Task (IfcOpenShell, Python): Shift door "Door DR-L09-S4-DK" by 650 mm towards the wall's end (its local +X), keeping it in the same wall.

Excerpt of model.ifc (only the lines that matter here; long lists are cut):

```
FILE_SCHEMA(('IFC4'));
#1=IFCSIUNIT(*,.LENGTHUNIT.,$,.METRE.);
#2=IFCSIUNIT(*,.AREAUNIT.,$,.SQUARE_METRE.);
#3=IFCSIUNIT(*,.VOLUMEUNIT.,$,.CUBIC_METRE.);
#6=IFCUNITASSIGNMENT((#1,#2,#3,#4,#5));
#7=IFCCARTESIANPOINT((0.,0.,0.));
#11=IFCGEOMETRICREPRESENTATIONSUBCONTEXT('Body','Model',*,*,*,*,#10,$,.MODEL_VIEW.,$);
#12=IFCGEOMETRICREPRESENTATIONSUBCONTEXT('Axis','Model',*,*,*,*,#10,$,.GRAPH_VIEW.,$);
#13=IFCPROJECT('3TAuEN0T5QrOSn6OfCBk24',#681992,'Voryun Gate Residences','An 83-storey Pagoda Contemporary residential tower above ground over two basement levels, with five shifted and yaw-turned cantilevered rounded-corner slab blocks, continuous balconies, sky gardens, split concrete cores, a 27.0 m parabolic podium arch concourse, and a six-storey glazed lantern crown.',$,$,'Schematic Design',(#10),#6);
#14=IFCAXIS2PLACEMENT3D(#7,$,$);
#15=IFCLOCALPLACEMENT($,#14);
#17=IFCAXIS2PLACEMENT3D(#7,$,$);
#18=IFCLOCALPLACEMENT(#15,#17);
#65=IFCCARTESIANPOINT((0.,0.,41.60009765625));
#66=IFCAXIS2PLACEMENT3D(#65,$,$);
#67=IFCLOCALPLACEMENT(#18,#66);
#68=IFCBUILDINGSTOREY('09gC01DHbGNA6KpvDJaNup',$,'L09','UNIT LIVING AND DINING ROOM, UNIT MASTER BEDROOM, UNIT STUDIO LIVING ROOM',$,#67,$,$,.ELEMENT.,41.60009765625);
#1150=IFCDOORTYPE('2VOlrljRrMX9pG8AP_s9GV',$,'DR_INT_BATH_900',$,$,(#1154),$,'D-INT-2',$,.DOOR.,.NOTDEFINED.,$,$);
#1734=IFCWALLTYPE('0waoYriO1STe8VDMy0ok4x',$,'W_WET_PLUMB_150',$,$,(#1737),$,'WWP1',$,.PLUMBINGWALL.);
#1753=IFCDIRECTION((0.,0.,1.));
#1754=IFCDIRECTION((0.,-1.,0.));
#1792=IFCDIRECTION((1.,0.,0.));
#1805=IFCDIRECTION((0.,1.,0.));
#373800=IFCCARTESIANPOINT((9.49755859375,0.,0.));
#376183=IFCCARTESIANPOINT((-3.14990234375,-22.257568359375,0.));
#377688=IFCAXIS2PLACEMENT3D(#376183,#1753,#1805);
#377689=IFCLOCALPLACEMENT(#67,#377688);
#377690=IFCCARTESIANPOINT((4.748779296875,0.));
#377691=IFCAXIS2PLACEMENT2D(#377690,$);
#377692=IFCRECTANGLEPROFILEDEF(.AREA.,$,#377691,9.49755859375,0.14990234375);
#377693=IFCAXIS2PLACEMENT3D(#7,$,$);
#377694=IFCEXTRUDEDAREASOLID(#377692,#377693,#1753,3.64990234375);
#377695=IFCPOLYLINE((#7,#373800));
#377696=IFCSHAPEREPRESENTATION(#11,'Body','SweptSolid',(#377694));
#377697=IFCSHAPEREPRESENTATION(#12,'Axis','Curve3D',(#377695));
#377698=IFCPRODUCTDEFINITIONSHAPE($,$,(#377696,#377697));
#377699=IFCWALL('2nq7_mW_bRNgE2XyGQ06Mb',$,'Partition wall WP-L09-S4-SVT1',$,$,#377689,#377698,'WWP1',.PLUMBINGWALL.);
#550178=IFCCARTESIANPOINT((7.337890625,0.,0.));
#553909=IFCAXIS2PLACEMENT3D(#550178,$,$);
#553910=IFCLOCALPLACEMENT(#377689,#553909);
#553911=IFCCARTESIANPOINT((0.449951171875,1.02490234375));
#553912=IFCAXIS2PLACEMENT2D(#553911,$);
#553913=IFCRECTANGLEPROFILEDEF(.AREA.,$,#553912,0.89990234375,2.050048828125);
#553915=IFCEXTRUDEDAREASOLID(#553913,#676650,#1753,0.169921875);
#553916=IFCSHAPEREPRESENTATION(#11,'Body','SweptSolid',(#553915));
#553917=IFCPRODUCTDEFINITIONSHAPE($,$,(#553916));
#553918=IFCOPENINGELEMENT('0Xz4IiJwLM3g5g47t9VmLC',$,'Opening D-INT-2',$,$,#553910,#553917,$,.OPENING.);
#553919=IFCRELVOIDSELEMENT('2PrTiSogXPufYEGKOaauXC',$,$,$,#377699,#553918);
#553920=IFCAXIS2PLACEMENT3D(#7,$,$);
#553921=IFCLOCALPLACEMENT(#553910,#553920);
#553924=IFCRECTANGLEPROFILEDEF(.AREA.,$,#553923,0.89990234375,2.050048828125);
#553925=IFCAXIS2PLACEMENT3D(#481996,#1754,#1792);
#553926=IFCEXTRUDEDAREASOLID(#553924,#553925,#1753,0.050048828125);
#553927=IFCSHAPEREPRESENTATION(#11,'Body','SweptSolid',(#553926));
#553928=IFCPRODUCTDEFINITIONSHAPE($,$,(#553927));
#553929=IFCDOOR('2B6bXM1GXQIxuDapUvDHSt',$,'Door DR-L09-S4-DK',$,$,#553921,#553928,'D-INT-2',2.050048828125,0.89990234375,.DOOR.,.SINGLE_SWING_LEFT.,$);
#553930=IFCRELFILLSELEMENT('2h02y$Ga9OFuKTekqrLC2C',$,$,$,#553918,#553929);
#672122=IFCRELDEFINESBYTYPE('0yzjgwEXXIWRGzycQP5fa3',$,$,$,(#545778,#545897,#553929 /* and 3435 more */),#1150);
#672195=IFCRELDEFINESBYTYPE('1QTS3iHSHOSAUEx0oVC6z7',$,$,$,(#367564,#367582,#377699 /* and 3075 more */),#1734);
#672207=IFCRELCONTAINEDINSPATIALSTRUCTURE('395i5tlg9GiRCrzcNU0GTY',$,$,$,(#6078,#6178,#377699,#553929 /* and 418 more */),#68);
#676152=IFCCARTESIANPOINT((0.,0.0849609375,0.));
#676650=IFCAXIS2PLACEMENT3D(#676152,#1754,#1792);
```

```python
import ifcopenshell
import ifcopenshell.api.geometry
import ifcopenshell.util.placement
import ifcopenshell.util.unit

model = ifcopenshell.open("model.ifc")
unit_scale = ifcopenshell.util.unit.calculate_unit_scale(model)

door = model.by_guid("2B6bXM1GXQIxuDapUvDHSt")
opening = door.FillsVoids[0].RelatingOpeningElement
wall = opening.VoidsElements[0].RelatingBuildingElement

wall_matrix = ifcopenshell.util.placement.get_local_placement(wall.ObjectPlacement)
shift = wall_matrix[:3, 0] * 0.65 / unit_scale
before = ifcopenshell.util.placement.get_local_placement(door.ObjectPlacement)[:3, 3].copy()

# The door is placed relative to its opening, so it follows when the opening moves.
matrix = ifcopenshell.util.placement.get_local_placement(opening.ObjectPlacement)
matrix[:3, 3] += shift
ifcopenshell.api.geometry.edit_object_placement(
    model, product=opening, matrix=matrix, is_si=False, should_transform_children=True
)

after = ifcopenshell.util.placement.get_local_placement(door.ObjectPlacement)[:3, 3]
print("door moved by", (after - before).round(3) + 0.0)

model.write("model-out.ifc")
```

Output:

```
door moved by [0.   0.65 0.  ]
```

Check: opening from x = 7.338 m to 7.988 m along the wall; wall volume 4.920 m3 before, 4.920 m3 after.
